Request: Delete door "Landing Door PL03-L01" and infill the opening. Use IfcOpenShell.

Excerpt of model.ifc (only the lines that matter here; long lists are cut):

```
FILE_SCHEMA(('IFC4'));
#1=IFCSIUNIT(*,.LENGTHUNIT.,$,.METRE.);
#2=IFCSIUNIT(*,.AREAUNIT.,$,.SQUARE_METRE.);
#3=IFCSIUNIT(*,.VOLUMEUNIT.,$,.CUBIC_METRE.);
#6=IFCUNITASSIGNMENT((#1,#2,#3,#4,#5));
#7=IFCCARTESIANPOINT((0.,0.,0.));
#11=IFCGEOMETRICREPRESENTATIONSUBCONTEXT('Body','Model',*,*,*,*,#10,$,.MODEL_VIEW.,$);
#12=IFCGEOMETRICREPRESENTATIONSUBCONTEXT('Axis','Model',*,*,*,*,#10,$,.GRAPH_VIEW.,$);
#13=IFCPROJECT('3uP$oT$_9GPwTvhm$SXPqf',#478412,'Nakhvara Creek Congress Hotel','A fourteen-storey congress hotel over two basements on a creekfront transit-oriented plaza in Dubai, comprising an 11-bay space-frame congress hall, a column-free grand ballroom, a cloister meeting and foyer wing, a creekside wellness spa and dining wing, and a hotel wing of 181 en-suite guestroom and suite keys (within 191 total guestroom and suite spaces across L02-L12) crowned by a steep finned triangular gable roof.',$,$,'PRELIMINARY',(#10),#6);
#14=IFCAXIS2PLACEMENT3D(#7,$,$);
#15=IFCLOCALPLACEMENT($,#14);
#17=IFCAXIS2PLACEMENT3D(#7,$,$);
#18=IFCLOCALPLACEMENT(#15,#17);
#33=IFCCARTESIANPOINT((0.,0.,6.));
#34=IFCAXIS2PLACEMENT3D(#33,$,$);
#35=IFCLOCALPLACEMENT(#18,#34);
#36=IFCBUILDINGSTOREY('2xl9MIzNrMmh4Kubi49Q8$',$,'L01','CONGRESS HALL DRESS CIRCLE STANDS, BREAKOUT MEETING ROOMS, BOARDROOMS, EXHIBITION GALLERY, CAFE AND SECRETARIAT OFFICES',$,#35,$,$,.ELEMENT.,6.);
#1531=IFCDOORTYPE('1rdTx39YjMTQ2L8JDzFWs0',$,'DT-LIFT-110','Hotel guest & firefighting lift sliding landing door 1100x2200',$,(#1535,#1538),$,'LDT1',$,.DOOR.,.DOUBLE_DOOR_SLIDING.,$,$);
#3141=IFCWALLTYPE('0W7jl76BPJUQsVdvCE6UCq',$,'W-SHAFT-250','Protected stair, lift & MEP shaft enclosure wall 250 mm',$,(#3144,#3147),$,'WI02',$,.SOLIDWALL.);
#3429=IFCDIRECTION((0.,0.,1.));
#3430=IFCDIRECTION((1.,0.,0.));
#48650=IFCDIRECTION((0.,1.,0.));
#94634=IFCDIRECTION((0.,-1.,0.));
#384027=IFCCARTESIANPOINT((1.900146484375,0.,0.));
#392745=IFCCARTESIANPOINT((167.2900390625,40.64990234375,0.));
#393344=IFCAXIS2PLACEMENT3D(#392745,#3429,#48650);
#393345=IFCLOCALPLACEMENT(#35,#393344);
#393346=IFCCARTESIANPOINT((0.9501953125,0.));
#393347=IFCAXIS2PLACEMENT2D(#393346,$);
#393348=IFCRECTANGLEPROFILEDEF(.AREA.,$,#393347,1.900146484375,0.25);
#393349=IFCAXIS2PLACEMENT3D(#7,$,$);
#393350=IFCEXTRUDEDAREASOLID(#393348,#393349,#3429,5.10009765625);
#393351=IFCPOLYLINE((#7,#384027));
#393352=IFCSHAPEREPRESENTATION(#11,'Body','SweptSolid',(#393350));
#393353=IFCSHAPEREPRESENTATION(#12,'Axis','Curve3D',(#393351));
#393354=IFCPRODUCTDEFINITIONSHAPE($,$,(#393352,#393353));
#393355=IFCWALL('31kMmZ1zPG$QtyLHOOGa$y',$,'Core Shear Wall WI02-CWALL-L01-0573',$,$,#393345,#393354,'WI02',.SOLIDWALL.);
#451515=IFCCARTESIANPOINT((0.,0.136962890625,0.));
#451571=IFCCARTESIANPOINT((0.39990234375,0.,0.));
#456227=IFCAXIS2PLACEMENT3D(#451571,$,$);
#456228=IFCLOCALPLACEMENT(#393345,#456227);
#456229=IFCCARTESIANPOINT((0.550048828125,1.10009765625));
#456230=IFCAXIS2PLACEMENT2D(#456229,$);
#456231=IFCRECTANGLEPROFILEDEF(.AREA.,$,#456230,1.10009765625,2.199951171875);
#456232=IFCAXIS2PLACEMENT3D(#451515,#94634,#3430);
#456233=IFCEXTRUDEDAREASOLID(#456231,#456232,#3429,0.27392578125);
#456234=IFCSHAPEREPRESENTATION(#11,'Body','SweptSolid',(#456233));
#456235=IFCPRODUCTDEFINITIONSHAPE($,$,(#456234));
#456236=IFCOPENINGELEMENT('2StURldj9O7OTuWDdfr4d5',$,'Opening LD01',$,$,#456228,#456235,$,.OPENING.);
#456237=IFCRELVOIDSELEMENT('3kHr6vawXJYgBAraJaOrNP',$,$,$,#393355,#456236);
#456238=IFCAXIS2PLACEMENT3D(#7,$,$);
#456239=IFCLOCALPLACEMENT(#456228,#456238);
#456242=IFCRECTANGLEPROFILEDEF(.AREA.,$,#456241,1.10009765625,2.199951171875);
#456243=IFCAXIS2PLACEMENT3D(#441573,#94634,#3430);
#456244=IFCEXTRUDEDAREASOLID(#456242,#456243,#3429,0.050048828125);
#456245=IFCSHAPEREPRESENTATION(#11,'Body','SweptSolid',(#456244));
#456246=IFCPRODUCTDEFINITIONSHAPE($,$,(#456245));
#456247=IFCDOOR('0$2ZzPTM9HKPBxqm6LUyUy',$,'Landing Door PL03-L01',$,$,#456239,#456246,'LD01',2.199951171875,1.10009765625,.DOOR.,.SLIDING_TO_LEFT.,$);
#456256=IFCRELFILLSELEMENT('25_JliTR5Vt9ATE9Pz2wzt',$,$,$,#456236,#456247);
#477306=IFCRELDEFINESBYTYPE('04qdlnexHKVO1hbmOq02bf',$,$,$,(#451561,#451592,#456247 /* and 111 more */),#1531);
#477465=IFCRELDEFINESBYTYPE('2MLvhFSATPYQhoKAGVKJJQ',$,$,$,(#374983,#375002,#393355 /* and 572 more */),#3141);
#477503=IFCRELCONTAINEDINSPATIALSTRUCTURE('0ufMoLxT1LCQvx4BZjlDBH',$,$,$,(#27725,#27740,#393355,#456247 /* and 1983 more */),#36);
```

```python
import ifcopenshell
import ifcopenshell.api.feature
import ifcopenshell.api.root
import ifcopenshell.geom
import ifcopenshell.util.shape

model = ifcopenshell.open("model.ifc")
settings = ifcopenshell.geom.settings()


def volume(element):
    """Net volume in cubic metres, openings subtracted."""
    shape = ifcopenshell.geom.create_shape(settings, element)
    return ifcopenshell.util.shape.get_volume(shape.geometry)


door = model.by_id(456247)
opening = door.FillsVoids[0].RelatingOpeningElement
wall = opening.VoidsElements[0].RelatingBuildingElement
before = volume(wall)

ifcopenshell.api.root.remove_product(model, product=door)
ifcopenshell.api.feature.remove_feature(model, feature=opening)

after = volume(wall)

print(f"wall volume {before:.3f} -> {after:.3f} m3")

model.write("model_rev.ifc")
```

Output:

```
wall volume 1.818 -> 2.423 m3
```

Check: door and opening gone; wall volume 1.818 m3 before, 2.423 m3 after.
